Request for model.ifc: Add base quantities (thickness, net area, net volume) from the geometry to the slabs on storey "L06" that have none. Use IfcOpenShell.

First a look at what the model holds.

```python
import ifcopenshell
import ifcopenshell.util.element
import ifcopenshell.util.unit

model = ifcopenshell.open("model.ifc")
print(model.schema)
for unit_type in ("LENGTHUNIT", "AREAUNIT", "VOLUMEUNIT"):
    print(unit_type, ifcopenshell.util.unit.calculate_unit_scale(model, unit_type))
storey = next(s for s in model.by_type("IfcBuildingStorey") if s.Name == "L06")
slabs = [e for e in ifcopenshell.util.element.get_decomposition(storey) if e.is_a("IfcSlab")]
for e in sorted(slabs, key=lambda e: e.id()):
    print(e.id(), e.is_a(), e.Name, list(ifcopenshell.util.element.get_psets(e, qtos_only=True)), sep=" | ")
```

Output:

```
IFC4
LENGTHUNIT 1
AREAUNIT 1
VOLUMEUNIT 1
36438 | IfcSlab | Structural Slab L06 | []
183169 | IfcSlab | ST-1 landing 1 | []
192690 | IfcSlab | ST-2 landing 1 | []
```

```python
import ifcopenshell
import ifcopenshell.api.pset
import ifcopenshell.geom
import ifcopenshell.util.element
import ifcopenshell.util.shape
import ifcopenshell.util.unit

model = ifcopenshell.open("model.ifc")
unit_scale = ifcopenshell.util.unit.calculate_unit_scale(model)
area_scale = ifcopenshell.util.unit.calculate_unit_scale(model, "AREAUNIT")
volume_scale = ifcopenshell.util.unit.calculate_unit_scale(model, "VOLUMEUNIT")
settings = ifcopenshell.geom.settings()

storey = next(s for s in model.by_type("IfcBuildingStorey") if s.Name == "L06")
slabs = [e for e in ifcopenshell.util.element.get_decomposition(storey) if e.is_a("IfcSlab")]

for e in sorted(slabs, key=lambda e: e.id()):
    if ifcopenshell.util.element.get_psets(e, qtos_only=True, should_inherit=False):
        continue
    # Geometry comes back in metres, in the element's own axes.
    shape = ifcopenshell.geom.create_shape(settings, e)
    values = {
        "Width": ifcopenshell.util.shape.get_z(shape.geometry) / unit_scale,
        "NetArea": ifcopenshell.util.shape.get_footprint_area(shape.geometry) / area_scale,
        "NetVolume": ifcopenshell.util.shape.get_volume(shape.geometry) / volume_scale,
    }
    qto = ifcopenshell.api.pset.add_qto(model, product=e, name="Qto_SlabBaseQuantities")
    ifcopenshell.api.pset.edit_qto(model, qto=qto, properties=values)
    print(e.id(), {k: round(v, 3) for k, v in values.items()})

model.write("model_rev.ifc")
```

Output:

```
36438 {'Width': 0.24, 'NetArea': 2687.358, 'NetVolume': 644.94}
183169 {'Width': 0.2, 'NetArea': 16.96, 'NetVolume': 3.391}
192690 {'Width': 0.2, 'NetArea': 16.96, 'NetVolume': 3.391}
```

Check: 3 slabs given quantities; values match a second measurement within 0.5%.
